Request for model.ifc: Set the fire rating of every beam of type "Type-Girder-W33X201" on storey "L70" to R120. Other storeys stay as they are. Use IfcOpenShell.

First a look at what the model holds.

```python
import ifcopenshell
import ifcopenshell.util.element

model = ifcopenshell.open("model.ifc")
print(model.schema)
storey = next(s for s in model.by_type("IfcBuildingStorey") if s.Name == "L70")
beams = [e for e in ifcopenshell.util.element.get_decomposition(storey) if e.is_a("IfcBeam")]
seen = {}
for e in beams:
    element_type = ifcopenshell.util.element.get_type(e)
    key = (element_type.Name if element_type != e and element_type else None, ifcopenshell.util.element.get_pset(e, "Pset_BeamCommon", "FireRating"))
    seen[key] = seen.get(key, 0) + 1
for (name, value), count in sorted(seen.items(), key=str):
    print(count, "x", name, "|", value)
```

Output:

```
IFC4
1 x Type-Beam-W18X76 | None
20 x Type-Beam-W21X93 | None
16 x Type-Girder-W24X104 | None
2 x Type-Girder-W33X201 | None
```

```python
import ifcopenshell
import ifcopenshell.api.pset
import ifcopenshell.util.element

model = ifcopenshell.open("model.ifc")

storey = next(s for s in model.by_type("IfcBuildingStorey") if s.Name == "L70")
beams = [e for e in ifcopenshell.util.element.get_decomposition(storey) if e.is_a("IfcBeam")]

count = 0
for e in beams:
    element_type = ifcopenshell.util.element.get_type(e)
    if element_type in (None, e) or element_type.Name != "Type-Girder-W33X201":
        continue
    # add_pset returns the element's existing set when there is one.
    pset = ifcopenshell.api.pset.add_pset(model, product=e, name="Pset_BeamCommon")
    ifcopenshell.api.pset.edit_pset(model, pset=pset, properties={"FireRating": "R120"})
    count += 1

print(count, "beams updated")

model.write("model-out.ifc")
```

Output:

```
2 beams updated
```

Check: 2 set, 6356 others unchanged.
